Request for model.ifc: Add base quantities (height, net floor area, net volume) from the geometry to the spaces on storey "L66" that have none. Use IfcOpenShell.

First a look at what the model holds.

```python
import ifcopenshell
import ifcopenshell.util.element
import ifcopenshell.util.unit

model = ifcopenshell.open("model.ifc")
print(model.schema)
for unit_type in ("LENGTHUNIT", "AREAUNIT", "VOLUMEUNIT"):
    print(unit_type, ifcopenshell.util.unit.calculate_unit_scale(model, unit_type))
storey = next(s for s in model.by_type("IfcBuildingStorey") if s.Name == "L66")
spaces = [e for e in ifcopenshell.util.element.get_decomposition(storey) if e.is_a("IfcSpace")]
for e in sorted(spaces, key=lambda e: e.id()):
    print(e.id(), e.is_a(), e.Name, list(ifcopenshell.util.element.get_psets(e, qtos_only=True)), sep=" | ")
```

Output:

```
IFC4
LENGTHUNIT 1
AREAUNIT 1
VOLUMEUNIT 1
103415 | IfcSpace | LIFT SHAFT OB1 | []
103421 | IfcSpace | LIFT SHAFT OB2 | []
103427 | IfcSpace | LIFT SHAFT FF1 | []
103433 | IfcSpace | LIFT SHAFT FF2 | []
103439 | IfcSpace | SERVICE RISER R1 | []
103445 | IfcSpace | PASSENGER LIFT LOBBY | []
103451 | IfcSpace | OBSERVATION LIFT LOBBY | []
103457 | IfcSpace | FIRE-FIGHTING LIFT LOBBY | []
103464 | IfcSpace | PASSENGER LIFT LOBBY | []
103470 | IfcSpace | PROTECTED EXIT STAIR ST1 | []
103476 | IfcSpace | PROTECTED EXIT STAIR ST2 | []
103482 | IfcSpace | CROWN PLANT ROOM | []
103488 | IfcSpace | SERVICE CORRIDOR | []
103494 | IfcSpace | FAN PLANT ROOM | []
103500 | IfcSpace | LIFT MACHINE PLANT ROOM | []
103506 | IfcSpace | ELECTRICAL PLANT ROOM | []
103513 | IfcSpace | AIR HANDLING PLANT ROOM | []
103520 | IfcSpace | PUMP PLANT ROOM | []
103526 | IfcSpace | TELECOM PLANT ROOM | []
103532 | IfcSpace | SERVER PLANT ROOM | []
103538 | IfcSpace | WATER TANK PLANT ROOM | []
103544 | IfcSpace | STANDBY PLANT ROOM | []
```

```python
import ifcopenshell
import ifcopenshell.api.pset
import ifcopenshell.geom
import ifcopenshell.util.element
import ifcopenshell.util.shape
import ifcopenshell.util.unit

model = ifcopenshell.open("model.ifc")
unit_scale = ifcopenshell.util.unit.calculate_unit_scale(model)
area_scale = ifcopenshell.util.unit.calculate_unit_scale(model, "AREAUNIT")
volume_scale = ifcopenshell.util.unit.calculate_unit_scale(model, "VOLUMEUNIT")
settings = ifcopenshell.geom.settings()

storey = next(s for s in model.by_type("IfcBuildingStorey") if s.Name == "L66")
spaces = [e for e in ifcopenshell.util.element.get_decomposition(storey) if e.is_a("IfcSpace")]

for e in sorted(spaces, key=lambda e: e.id()):
    if ifcopenshell.util.element.get_psets(e, qtos_only=True, should_inherit=False):
        continue
    # Geometry comes back in metres, in the element's own axes.
    shape = ifcopenshell.geom.create_shape(settings, e)
    values = {
        "Height": ifcopenshell.util.shape.get_z(shape.geometry) / unit_scale,
        "NetFloorArea": ifcopenshell.util.shape.get_footprint_area(shape.geometry) / area_scale,
        "NetVolume": ifcopenshell.util.shape.get_volume(shape.geometry) / volume_scale,
    }
    qto = ifcopenshell.api.pset.add_qto(model, product=e, name="Qto_SpaceBaseQuantities")
    ifcopenshell.api.pset.edit_qto(model, qto=qto, properties=values)
    print(e.id(), {k: round(v, 3) for k, v in values.items()})

model.write("model_edited.ifc")
```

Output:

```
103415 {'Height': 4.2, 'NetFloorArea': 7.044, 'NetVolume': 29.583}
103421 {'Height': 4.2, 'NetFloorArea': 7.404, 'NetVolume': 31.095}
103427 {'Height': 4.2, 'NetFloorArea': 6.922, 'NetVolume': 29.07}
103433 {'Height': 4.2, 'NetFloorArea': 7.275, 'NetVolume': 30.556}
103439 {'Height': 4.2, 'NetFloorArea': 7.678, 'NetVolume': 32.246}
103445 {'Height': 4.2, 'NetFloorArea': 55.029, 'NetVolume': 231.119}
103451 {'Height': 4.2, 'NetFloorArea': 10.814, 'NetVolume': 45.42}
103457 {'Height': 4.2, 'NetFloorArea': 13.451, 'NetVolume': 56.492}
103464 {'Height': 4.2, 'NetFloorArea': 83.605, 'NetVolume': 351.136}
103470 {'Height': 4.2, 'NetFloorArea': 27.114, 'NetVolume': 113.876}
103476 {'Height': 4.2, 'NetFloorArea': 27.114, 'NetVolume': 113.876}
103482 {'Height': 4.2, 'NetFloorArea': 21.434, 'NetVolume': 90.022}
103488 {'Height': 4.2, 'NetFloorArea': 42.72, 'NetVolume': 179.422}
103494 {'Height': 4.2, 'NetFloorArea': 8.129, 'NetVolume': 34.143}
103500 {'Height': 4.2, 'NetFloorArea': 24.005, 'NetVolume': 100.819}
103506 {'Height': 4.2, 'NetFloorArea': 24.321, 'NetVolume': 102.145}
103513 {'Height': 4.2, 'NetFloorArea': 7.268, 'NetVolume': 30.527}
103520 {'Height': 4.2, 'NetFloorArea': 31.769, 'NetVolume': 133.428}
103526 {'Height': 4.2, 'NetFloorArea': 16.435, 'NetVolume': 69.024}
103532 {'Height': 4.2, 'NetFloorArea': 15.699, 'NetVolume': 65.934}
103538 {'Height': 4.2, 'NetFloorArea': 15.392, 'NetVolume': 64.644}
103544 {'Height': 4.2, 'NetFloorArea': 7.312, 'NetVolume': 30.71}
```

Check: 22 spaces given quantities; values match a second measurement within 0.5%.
